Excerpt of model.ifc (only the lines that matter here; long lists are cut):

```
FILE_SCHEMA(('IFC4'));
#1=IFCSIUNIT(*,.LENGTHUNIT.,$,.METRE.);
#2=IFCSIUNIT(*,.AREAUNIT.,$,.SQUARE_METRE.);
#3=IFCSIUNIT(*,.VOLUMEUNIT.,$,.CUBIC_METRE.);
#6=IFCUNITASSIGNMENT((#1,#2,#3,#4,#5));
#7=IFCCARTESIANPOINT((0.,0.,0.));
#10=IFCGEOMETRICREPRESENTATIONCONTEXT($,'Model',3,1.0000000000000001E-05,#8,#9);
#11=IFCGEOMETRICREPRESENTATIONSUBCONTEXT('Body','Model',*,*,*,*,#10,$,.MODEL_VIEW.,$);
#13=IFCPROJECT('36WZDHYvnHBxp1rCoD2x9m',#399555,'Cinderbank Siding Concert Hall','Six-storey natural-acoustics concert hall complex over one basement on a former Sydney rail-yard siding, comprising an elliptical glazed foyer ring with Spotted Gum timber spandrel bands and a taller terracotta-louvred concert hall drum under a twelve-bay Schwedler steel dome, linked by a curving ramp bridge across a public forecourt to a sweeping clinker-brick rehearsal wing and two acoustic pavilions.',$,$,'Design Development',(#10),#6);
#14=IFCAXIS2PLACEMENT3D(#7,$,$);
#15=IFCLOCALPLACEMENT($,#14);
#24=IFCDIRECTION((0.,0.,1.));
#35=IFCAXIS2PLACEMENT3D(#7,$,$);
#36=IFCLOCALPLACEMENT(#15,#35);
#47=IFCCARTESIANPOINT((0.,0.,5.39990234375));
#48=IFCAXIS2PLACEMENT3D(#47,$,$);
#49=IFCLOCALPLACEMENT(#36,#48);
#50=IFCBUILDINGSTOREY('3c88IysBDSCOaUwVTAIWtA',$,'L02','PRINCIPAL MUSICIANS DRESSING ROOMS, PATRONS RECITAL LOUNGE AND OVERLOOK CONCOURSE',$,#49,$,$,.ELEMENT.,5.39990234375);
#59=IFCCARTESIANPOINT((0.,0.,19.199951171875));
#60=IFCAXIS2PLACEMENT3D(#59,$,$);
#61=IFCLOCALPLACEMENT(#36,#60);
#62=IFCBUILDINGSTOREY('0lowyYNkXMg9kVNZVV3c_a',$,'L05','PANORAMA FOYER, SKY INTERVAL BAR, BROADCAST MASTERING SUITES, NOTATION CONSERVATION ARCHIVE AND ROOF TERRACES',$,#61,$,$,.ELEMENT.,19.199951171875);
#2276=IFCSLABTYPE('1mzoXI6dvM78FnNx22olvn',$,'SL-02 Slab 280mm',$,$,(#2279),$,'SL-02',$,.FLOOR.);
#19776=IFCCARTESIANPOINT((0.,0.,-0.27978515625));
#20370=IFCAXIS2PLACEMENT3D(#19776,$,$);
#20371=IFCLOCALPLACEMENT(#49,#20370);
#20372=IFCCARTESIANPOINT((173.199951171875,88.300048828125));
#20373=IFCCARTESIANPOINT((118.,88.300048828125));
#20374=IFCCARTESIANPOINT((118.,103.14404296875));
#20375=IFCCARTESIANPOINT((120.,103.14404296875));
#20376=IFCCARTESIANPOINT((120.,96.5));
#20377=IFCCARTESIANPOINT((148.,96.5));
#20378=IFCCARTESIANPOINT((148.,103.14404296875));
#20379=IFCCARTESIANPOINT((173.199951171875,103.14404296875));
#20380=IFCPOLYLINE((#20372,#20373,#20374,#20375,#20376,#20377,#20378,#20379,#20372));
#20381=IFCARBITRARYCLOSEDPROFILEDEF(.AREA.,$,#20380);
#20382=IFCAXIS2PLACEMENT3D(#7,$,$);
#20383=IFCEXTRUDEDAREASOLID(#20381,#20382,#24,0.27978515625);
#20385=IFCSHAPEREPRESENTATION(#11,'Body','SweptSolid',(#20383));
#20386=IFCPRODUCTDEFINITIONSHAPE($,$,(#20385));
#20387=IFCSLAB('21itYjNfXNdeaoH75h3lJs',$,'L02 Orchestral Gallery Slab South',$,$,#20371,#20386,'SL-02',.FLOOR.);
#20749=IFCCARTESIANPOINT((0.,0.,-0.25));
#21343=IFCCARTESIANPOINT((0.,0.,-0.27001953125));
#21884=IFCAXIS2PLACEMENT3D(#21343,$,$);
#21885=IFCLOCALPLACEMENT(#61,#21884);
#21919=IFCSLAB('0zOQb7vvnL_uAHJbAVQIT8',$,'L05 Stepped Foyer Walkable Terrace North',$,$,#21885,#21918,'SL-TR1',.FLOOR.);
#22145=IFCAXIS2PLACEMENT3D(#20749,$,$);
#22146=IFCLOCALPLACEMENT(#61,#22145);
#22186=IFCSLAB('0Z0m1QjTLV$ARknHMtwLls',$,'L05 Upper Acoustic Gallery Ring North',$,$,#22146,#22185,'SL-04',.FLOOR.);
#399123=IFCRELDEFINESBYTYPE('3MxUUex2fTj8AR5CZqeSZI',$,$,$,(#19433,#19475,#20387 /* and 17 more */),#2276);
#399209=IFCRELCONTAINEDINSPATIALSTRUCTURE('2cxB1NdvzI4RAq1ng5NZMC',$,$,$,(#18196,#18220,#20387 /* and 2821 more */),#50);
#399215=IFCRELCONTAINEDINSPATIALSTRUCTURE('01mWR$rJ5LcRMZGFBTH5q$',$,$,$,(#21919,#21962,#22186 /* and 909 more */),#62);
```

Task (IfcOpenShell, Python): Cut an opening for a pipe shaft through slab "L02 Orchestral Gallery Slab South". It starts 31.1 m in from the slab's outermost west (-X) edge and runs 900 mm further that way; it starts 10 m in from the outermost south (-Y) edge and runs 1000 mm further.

```python
import numpy as np
import ifcopenshell
import ifcopenshell.api.feature
import ifcopenshell.api.geometry
import ifcopenshell.api.root
import ifcopenshell.geom
import ifcopenshell.util.placement
import ifcopenshell.util.representation
import ifcopenshell.util.shape
import ifcopenshell.util.unit

model = ifcopenshell.open("model.ifc")
unit_scale = ifcopenshell.util.unit.calculate_unit_scale(model)
settings = ifcopenshell.geom.settings()


def volume(element):
    """Net volume in cubic metres, openings subtracted."""
    shape = ifcopenshell.geom.create_shape(settings, element)
    return ifcopenshell.util.shape.get_volume(shape.geometry)


slab = model.by_guid("21itYjNfXNdeaoH75h3lJs")
before = volume(slab)

# Extent in the slab's own axes, in metres. The edges named are its -X and -Y sides.
slab_shape = ifcopenshell.geom.create_shape(settings, slab)
vertices = ifcopenshell.util.shape.get_vertices(slab_shape.geometry)
x_min, y_min, bottom = vertices.min(axis=0)
top = vertices[:, 2].max()

opening = ifcopenshell.api.root.create_entity(model, ifc_class="IfcOpeningElement", name="Pipe shaft opening", predefined_type="OPENING")
context = ifcopenshell.util.representation.get_context(model, "Model", "Body", "MODEL_VIEW")
width, depth = 0.9, 1
outline = [(0.0, 0.0), (width, 0.0), (width, depth), (0.0, depth), (0.0, 0.0)]
# Overshoot both faces by 50 mm so the cut is clean.
shape = ifcopenshell.api.geometry.add_slab_representation(
    model, context=context, depth=top - bottom + 0.1, polyline=outline
)
ifcopenshell.api.geometry.assign_representation(model, product=opening, representation=shape)

matrix = ifcopenshell.util.placement.get_local_placement(slab.ObjectPlacement)
matrix[:, 3] = matrix @ np.append(np.array([x_min + 31.1, y_min + 10, bottom - 0.05]) / unit_scale, 1.0)
ifcopenshell.api.geometry.edit_object_placement(model, product=opening, matrix=matrix, is_si=False)
ifcopenshell.api.feature.add_feature(model, feature=opening, element=slab)

after = volume(slab)

print(f"slab volume {before:.3f} -> {after:.3f} m3")

model.write("model_rev.ifc")
```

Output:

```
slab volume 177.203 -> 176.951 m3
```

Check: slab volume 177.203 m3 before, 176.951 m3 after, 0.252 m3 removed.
